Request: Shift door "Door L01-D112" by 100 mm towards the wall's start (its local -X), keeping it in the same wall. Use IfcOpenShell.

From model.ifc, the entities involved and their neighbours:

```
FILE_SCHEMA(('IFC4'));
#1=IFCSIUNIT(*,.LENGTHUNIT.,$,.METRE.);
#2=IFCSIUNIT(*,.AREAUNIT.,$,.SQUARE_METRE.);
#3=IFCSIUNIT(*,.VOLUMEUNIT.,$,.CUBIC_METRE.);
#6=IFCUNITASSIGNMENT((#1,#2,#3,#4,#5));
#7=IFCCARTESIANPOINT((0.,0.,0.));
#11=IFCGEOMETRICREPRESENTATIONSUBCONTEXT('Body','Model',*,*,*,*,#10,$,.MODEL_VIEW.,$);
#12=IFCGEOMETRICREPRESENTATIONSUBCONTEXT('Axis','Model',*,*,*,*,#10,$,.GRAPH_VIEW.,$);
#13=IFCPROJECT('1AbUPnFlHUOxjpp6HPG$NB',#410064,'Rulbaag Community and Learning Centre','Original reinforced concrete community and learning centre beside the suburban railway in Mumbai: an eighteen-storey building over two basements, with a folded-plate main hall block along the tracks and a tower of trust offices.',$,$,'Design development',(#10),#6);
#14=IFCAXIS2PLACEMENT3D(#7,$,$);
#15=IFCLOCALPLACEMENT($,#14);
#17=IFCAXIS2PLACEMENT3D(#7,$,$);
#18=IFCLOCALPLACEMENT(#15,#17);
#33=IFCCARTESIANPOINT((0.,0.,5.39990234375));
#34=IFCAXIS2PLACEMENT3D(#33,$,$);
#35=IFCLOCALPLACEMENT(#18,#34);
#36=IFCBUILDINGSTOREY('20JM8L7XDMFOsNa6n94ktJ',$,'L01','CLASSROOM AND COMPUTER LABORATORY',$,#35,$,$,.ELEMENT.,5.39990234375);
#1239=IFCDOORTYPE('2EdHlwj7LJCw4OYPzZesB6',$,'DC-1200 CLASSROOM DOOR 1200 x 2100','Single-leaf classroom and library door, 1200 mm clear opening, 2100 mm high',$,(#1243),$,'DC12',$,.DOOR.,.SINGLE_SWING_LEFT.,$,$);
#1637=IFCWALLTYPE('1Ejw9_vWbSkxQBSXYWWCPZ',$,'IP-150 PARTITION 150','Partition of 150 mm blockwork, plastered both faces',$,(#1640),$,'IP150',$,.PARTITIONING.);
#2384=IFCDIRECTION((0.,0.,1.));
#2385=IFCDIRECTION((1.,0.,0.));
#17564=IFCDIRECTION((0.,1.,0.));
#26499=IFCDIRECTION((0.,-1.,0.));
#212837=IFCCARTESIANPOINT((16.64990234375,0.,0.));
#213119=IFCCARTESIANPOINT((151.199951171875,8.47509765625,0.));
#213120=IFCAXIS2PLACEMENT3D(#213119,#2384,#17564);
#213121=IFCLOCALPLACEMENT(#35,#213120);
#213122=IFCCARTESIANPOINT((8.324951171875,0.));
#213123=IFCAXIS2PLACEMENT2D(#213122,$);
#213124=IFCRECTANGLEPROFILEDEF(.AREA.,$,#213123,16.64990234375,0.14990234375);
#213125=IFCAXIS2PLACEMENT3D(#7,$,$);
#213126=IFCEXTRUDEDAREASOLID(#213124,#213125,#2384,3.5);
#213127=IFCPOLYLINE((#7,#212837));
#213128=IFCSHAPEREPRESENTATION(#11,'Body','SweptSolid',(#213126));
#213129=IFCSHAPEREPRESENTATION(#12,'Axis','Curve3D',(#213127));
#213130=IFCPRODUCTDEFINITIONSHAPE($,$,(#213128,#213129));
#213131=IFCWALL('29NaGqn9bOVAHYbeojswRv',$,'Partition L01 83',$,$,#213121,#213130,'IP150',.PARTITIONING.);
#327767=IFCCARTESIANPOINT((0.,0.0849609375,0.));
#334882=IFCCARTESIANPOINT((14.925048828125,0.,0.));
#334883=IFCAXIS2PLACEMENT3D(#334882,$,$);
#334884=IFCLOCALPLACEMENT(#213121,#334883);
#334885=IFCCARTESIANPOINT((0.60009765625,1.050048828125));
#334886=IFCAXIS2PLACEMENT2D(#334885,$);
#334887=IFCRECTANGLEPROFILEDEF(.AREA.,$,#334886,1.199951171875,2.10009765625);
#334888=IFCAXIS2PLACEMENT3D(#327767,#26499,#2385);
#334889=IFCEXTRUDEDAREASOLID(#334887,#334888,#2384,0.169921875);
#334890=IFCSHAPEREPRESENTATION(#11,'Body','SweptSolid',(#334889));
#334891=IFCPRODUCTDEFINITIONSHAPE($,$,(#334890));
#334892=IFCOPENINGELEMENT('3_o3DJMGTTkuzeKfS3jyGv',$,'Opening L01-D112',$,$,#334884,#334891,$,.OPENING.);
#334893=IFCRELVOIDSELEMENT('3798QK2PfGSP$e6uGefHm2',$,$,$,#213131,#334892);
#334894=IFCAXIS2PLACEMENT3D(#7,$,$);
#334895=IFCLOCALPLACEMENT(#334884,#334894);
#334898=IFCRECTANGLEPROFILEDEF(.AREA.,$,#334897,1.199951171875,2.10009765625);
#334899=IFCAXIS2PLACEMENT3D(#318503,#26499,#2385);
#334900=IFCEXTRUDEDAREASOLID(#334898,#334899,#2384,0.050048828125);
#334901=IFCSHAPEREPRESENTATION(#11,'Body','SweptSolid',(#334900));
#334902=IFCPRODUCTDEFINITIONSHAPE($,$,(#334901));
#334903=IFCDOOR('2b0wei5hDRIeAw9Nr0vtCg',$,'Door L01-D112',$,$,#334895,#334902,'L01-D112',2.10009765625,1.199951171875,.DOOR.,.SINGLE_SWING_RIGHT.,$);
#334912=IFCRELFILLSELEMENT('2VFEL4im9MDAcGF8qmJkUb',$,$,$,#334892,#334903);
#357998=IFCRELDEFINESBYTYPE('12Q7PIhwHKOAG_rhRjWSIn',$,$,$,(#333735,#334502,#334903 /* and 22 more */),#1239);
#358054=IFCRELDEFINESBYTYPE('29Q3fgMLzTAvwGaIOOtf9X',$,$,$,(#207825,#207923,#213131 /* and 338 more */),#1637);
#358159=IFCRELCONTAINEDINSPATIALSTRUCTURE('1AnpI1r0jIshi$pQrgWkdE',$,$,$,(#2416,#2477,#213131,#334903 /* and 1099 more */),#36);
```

```python
import ifcopenshell
import ifcopenshell.api.geometry
import ifcopenshell.util.placement
import ifcopenshell.util.unit

model = ifcopenshell.open("model.ifc")
unit_scale = ifcopenshell.util.unit.calculate_unit_scale(model)

door = model.by_id(334903)
opening = door.FillsVoids[0].RelatingOpeningElement
wall = opening.VoidsElements[0].RelatingBuildingElement

wall_matrix = ifcopenshell.util.placement.get_local_placement(wall.ObjectPlacement)
shift = wall_matrix[:3, 0] * -0.1 / unit_scale
before = ifcopenshell.util.placement.get_local_placement(door.ObjectPlacement)[:3, 3].copy()

# The door is placed relative to its opening, so it follows when the opening moves.
matrix = ifcopenshell.util.placement.get_local_placement(opening.ObjectPlacement)
matrix[:3, 3] += shift
ifcopenshell.api.geometry.edit_object_placement(
    model, product=opening, matrix=matrix, is_si=False, should_transform_children=True
)

after = ifcopenshell.util.placement.get_local_placement(door.ObjectPlacement)[:3, 3]
print("door moved by", (after - before).round(3) + 0.0)

model.write("model-out.ifc")
```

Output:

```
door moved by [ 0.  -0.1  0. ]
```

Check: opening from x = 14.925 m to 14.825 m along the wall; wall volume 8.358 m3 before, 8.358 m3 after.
